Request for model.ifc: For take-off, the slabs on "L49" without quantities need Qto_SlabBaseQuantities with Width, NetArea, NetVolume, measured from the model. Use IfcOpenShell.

First a look at what the model holds.

```python
import ifcopenshell
import ifcopenshell.util.element
import ifcopenshell.util.unit

model = ifcopenshell.open("model.ifc")
print(model.schema)
for unit_type in ("LENGTHUNIT", "AREAUNIT", "VOLUMEUNIT"):
    print(unit_type, ifcopenshell.util.unit.calculate_unit_scale(model, unit_type))
storey = next(s for s in model.by_type("IfcBuildingStorey") if s.Name == "L49")
slabs = [e for e in ifcopenshell.util.element.get_decomposition(storey) if e.is_a("IfcSlab")]
for e in sorted(slabs, key=lambda e: e.id()):
    print(e.id(), e.is_a(), e.Name, list(ifcopenshell.util.element.get_psets(e, qtos_only=True)), sep=" | ")
```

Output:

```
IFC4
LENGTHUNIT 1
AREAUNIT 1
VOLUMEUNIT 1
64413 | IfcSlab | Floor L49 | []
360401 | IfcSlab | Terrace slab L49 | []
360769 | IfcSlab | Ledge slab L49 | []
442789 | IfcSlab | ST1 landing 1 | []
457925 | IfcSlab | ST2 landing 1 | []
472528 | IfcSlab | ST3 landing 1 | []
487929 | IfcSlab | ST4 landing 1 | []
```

```python
import ifcopenshell
import ifcopenshell.api.pset
import ifcopenshell.geom
import ifcopenshell.util.element
import ifcopenshell.util.shape
import ifcopenshell.util.unit

model = ifcopenshell.open("model.ifc")
unit_scale = ifcopenshell.util.unit.calculate_unit_scale(model)
area_scale = ifcopenshell.util.unit.calculate_unit_scale(model, "AREAUNIT")
volume_scale = ifcopenshell.util.unit.calculate_unit_scale(model, "VOLUMEUNIT")
settings = ifcopenshell.geom.settings()

storey = next(s for s in model.by_type("IfcBuildingStorey") if s.Name == "L49")
slabs = [e for e in ifcopenshell.util.element.get_decomposition(storey) if e.is_a("IfcSlab")]

for e in sorted(slabs, key=lambda e: e.id()):
    if ifcopenshell.util.element.get_psets(e, qtos_only=True, should_inherit=False):
        continue
    # Geometry comes back in metres, in the element's own axes.
    shape = ifcopenshell.geom.create_shape(settings, e)
    values = {
        "Width": ifcopenshell.util.shape.get_z(shape.geometry) / unit_scale,
        "NetArea": ifcopenshell.util.shape.get_footprint_area(shape.geometry) / area_scale,
        "NetVolume": ifcopenshell.util.shape.get_volume(shape.geometry) / volume_scale,
    }
    qto = ifcopenshell.api.pset.add_qto(model, product=e, name="Qto_SlabBaseQuantities")
    ifcopenshell.api.pset.edit_qto(model, qto=qto, properties=values)
    print(e.id(), {k: round(v, 3) for k, v in values.items()})

model.write("model-out.ifc")
```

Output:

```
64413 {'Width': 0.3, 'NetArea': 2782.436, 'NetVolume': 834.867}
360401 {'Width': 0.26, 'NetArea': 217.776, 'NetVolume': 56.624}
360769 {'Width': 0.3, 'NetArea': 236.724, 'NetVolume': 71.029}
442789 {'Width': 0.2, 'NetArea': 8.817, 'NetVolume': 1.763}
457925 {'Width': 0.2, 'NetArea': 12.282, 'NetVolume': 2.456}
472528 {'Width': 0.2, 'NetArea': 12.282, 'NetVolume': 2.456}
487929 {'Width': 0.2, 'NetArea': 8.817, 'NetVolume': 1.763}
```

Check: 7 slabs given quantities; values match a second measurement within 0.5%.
